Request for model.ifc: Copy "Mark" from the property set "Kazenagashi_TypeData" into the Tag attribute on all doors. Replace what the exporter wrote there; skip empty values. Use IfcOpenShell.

First a look at what the model holds.

```python
import ifcopenshell
import ifcopenshell.util.element

model = ifcopenshell.open("model.ifc")
print(model.schema)
doors = model.by_type("IfcDoor")
print(len(doors), "doors")
for e in doors[:8]:
    source = ifcopenshell.util.element.get_pset(e, "Kazenagashi_TypeData", "Mark")
    target = e.Tag
    print(e.id(), repr(source), repr(target), sep=" | ")
```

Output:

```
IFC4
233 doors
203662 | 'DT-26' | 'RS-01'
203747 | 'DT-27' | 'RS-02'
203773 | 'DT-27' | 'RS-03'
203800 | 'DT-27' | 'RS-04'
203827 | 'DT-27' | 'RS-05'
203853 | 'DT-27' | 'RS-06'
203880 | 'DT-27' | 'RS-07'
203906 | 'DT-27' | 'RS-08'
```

```python
import ifcopenshell
import ifcopenshell.util.element

model = ifcopenshell.open("model.ifc")

count = 0
for e in model.by_type("IfcDoor"):
    value = ifcopenshell.util.element.get_pset(e, "Kazenagashi_TypeData", "Mark")
    current = e.Tag
    if not value or not value.strip() or current == value:
        continue
    e.Tag = value
    count += 1

print(count, "doors updated")

model.write("model_edited.ifc")
```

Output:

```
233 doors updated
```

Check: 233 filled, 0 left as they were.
